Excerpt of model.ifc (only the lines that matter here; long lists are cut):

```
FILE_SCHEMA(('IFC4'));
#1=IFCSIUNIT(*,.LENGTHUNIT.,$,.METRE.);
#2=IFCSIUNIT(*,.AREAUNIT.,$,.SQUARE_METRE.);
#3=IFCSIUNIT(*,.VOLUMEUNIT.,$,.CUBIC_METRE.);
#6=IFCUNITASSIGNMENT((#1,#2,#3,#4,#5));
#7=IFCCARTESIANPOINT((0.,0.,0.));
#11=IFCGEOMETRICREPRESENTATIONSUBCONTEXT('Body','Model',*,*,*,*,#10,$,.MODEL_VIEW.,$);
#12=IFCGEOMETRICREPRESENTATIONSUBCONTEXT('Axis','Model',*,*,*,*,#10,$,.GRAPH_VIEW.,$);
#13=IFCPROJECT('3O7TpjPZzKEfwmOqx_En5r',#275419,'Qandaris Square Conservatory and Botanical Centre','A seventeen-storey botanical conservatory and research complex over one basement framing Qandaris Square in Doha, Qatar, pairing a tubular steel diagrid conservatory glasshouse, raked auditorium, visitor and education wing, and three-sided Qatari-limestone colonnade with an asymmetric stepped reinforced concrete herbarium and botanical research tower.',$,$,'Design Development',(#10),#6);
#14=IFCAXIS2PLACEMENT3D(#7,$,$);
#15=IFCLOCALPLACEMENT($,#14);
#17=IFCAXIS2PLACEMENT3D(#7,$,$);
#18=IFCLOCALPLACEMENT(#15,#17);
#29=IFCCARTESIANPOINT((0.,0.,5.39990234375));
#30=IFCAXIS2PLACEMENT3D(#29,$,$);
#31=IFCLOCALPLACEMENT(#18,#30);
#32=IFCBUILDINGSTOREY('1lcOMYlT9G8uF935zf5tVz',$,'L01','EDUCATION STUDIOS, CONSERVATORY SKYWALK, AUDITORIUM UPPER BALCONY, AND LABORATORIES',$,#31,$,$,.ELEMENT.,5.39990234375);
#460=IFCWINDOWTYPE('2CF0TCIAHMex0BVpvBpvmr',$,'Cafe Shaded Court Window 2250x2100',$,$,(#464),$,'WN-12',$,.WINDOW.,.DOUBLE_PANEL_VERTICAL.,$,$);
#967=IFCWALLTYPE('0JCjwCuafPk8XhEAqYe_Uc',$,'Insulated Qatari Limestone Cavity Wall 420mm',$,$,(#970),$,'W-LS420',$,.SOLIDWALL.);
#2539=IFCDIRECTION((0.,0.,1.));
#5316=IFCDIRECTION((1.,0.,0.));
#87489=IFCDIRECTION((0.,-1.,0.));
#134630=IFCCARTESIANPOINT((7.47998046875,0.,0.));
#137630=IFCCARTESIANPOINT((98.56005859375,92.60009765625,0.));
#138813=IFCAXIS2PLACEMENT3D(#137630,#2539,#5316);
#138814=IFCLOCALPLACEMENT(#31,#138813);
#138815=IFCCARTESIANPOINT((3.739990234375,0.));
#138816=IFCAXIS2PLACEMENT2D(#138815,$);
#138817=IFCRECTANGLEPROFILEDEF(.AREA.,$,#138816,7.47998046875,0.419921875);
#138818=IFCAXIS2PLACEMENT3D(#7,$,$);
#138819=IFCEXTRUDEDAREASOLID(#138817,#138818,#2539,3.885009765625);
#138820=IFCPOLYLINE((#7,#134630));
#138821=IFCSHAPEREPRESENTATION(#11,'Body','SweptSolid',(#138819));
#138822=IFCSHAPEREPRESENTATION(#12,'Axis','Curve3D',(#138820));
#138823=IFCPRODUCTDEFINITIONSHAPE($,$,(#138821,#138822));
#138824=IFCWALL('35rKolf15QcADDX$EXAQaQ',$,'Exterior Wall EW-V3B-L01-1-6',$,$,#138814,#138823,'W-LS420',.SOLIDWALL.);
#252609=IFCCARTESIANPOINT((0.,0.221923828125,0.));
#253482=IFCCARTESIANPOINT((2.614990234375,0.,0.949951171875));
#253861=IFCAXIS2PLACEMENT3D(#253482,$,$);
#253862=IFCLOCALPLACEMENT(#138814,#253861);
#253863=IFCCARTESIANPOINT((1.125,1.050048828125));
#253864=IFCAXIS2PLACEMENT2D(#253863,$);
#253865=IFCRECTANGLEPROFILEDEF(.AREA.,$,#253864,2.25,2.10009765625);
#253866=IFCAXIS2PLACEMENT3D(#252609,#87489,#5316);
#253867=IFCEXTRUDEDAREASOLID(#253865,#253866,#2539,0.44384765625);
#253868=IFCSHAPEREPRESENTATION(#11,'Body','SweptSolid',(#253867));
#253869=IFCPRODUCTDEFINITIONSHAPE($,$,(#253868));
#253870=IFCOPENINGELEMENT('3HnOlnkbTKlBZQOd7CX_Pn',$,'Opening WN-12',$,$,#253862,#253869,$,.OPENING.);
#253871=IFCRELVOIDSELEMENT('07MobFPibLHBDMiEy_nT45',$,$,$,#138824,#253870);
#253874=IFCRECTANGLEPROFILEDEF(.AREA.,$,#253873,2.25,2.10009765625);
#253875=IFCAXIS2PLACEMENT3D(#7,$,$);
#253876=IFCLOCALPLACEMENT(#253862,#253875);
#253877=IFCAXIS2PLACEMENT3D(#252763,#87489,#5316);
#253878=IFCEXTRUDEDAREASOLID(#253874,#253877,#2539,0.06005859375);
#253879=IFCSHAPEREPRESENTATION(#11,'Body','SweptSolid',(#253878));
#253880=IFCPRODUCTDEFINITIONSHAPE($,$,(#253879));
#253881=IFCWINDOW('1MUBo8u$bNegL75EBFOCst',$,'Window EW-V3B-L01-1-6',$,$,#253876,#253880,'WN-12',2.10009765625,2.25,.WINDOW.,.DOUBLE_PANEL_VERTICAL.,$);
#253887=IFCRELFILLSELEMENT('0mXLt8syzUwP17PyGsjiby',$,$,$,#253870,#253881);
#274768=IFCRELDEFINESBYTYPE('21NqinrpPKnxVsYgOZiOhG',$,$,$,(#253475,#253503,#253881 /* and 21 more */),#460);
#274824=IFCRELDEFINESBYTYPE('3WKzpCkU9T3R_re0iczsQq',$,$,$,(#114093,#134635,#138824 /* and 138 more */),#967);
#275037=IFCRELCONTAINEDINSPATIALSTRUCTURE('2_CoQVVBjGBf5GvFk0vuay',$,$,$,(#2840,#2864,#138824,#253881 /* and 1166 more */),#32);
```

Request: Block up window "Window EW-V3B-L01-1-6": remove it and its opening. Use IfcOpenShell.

```python
import ifcopenshell
import ifcopenshell.api.feature
import ifcopenshell.api.root
import ifcopenshell.geom
import ifcopenshell.util.shape

model = ifcopenshell.open("model.ifc")
settings = ifcopenshell.geom.settings()


def volume(element):
    """Net volume in cubic metres, openings subtracted."""
    shape = ifcopenshell.geom.create_shape(settings, element)
    return ifcopenshell.util.shape.get_volume(shape.geometry)


window = model.by_guid("1MUBo8u$bNegL75EBFOCst")
opening = window.FillsVoids[0].RelatingOpeningElement
wall = opening.VoidsElements[0].RelatingBuildingElement
before = volume(wall)

ifcopenshell.api.root.remove_product(model, product=window)
ifcopenshell.api.feature.remove_feature(model, feature=opening)

after = volume(wall)

print(f"wall volume {before:.3f} -> {after:.3f} m3")

model.write("model_edited.ifc")
```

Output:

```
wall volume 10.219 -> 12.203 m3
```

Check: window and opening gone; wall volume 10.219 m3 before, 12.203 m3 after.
